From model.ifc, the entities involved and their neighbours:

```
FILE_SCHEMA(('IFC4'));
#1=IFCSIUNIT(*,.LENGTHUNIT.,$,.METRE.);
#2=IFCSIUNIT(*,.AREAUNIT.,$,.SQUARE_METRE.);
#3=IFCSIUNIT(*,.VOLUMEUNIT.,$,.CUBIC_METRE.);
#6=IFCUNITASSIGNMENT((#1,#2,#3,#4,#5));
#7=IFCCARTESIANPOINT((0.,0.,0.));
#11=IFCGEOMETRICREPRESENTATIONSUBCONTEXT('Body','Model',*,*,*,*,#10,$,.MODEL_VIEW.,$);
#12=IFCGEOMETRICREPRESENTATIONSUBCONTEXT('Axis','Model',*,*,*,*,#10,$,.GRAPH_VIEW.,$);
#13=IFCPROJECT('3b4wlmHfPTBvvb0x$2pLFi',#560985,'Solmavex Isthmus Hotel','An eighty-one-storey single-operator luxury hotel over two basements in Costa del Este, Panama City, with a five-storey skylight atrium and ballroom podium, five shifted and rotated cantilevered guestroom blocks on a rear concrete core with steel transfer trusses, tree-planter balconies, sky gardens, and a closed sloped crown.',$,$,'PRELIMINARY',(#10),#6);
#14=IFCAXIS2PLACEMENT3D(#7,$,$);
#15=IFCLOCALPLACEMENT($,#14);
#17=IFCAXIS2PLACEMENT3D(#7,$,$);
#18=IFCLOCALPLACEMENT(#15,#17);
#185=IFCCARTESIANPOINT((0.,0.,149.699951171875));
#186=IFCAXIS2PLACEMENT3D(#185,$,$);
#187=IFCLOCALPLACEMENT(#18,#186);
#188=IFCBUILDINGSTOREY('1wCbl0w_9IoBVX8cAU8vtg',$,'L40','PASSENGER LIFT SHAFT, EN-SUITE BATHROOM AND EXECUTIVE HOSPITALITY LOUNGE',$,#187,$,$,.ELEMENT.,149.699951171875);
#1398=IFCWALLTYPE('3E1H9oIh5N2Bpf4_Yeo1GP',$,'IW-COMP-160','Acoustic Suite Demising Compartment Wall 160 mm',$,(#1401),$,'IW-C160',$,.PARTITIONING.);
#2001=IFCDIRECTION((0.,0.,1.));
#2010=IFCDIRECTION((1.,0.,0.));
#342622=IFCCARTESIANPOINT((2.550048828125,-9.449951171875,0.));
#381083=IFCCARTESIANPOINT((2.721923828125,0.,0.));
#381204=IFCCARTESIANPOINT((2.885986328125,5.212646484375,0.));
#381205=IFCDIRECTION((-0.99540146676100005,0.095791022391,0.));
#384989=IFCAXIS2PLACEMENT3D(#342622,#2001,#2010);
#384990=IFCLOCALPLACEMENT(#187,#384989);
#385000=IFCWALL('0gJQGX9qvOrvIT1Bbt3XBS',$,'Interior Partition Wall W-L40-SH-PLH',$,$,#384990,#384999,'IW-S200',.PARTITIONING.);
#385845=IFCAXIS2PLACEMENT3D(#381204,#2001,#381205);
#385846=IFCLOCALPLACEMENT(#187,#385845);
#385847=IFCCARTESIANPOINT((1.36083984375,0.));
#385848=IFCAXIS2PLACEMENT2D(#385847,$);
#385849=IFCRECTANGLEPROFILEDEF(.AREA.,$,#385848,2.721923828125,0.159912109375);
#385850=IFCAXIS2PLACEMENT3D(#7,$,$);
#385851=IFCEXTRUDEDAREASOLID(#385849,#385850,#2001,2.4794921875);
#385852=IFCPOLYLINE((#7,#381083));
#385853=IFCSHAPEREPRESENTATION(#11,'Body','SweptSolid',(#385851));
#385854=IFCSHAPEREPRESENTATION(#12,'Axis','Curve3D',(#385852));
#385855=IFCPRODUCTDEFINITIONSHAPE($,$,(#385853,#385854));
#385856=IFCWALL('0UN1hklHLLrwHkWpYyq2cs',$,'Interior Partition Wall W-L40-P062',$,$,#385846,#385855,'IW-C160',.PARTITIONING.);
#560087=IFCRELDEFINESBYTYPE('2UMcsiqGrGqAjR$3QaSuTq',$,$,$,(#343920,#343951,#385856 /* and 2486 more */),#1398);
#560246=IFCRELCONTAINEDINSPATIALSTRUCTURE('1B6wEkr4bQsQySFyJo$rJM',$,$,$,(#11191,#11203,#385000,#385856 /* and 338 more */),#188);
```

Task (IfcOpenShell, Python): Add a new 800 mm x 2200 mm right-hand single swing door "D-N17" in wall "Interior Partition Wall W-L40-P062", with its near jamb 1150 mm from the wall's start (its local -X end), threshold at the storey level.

```python
import numpy as np
import ifcopenshell
import ifcopenshell.api.feature
import ifcopenshell.api.geometry
import ifcopenshell.api.root
import ifcopenshell.api.spatial
import ifcopenshell.geom
import ifcopenshell.util.element
import ifcopenshell.util.placement
import ifcopenshell.util.representation
import ifcopenshell.util.shape
import ifcopenshell.util.unit

model = ifcopenshell.open("model.ifc")
unit_scale = ifcopenshell.util.unit.calculate_unit_scale(model)
settings = ifcopenshell.geom.settings()


def volume(element):
    """Net volume in cubic metres, openings subtracted."""
    shape = ifcopenshell.geom.create_shape(settings, element)
    return ifcopenshell.util.shape.get_volume(shape.geometry)


wall = model.by_guid("0UN1hklHLLrwHkWpYyq2cs")
storey = ifcopenshell.util.element.get_container(wall, ifc_class="IfcBuildingStorey")
context = ifcopenshell.util.representation.get_context(model, "Model", "Body", "MODEL_VIEW")
before = volume(wall)

width, height, from_end, sill = 0.8, 2.2, 1.15, 0.0  # metres

# The wall runs along its own X axis, and the end named is its -X end.
wall_shape = ifcopenshell.geom.create_shape(settings, wall)
x, y, z = ifcopenshell.util.shape.get_vertices(wall_shape.geometry).T
start = x.min() + from_end
face, thickness = float(y.min()), float(y.max() - y.min())
wall_matrix = ifcopenshell.util.placement.get_local_placement(wall.ObjectPlacement)
level = ifcopenshell.util.placement.get_local_placement(storey.ObjectPlacement)[2, 3]


def in_wall(x, y):
    """Placement at x, y metres in the wall's axes, at sill height."""
    matrix = wall_matrix.copy()
    matrix[:, 3] = wall_matrix @ np.array([x / unit_scale, y / unit_scale, 0.0, 1.0])
    matrix[2, 3] = level + sill / unit_scale
    return matrix


# Opening: a box that overshoots both wall faces by 50 mm.
opening = ifcopenshell.api.root.create_entity(model, ifc_class="IfcOpeningElement", predefined_type="OPENING")
box = ifcopenshell.api.geometry.add_wall_representation(
    model, context=context, length=width, height=height, thickness=thickness + 0.1
)
ifcopenshell.api.geometry.assign_representation(model, product=opening, representation=box)
ifcopenshell.api.geometry.edit_object_placement(model, product=opening, matrix=in_wall(start, face - 0.05), is_si=False)
ifcopenshell.api.feature.add_feature(model, feature=opening, element=wall)

door = ifcopenshell.api.root.create_entity(model, ifc_class="IfcDoor", name="D-N17", predefined_type="DOOR")
door.OverallWidth, door.OverallHeight = width / unit_scale, height / unit_scale
door.OperationType = "SINGLE_SWING_RIGHT"
body = ifcopenshell.api.geometry.add_door_representation(
    model,
    context=context,
    overall_width=door.OverallWidth,
    overall_height=door.OverallHeight,
    operation_type="SINGLE_SWING_RIGHT",
    lining_properties={"LiningDepth": thickness / unit_scale, "ThresholdDepth": thickness / unit_scale},
)
ifcopenshell.api.geometry.assign_representation(model, product=door, representation=body)
ifcopenshell.api.spatial.assign_container(model, products=[door], relating_structure=storey)
ifcopenshell.api.feature.add_filling(model, opening=opening, element=door)

# The lining spans the wall, so the door starts at the wall face.
ifcopenshell.api.geometry.edit_object_placement(model, product=door, matrix=in_wall(start, face), is_si=False)

after = volume(wall)

print(f"wall volume {before:.3f} -> {after:.3f} m3")

model.write("model_updated.ifc")
```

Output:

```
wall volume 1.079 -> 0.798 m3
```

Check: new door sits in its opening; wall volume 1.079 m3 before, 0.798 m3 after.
